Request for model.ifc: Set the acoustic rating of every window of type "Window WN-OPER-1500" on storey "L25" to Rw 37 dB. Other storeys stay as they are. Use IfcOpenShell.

First a look at what the model holds.

```python
import ifcopenshell
import ifcopenshell.util.element

model = ifcopenshell.open("model.ifc")
print(model.schema)
storey = next(s for s in model.by_type("IfcBuildingStorey") if s.Name == "L25")
windows = [e for e in ifcopenshell.util.element.get_decomposition(storey) if e.is_a("IfcWindow")]
seen = {}
for e in windows:
    element_type = ifcopenshell.util.element.get_type(e)
    key = (element_type.Name if element_type != e and element_type else None, ifcopenshell.util.element.get_pset(e, "Pset_WindowCommon", "AcousticRating"))
    seen[key] = seen.get(key, 0) + 1
for (name, value), count in sorted(seen.items(), key=str):
    print(count, "x", name, "|", value)
```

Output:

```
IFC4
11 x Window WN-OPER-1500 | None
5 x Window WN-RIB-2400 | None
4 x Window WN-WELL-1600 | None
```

```python
import ifcopenshell
import ifcopenshell.api.pset
import ifcopenshell.util.element

model = ifcopenshell.open("model.ifc")

storey = next(s for s in model.by_type("IfcBuildingStorey") if s.Name == "L25")
windows = [e for e in ifcopenshell.util.element.get_decomposition(storey) if e.is_a("IfcWindow")]

count = 0
for e in windows:
    element_type = ifcopenshell.util.element.get_type(e)
    if element_type in (None, e) or element_type.Name != "Window WN-OPER-1500":
        continue
    found = ifcopenshell.util.element.get_pset(e, "Pset_WindowCommon", should_inherit=False)
    if found:
        pset = model.by_id(found["id"])
        if len(ifcopenshell.util.element.get_elements_by_pset(pset)) > 1:
            pset = ifcopenshell.api.pset.unshare_pset(model, products=[e], pset=pset)[0]
    else:
        pset = ifcopenshell.api.pset.add_pset(model, product=e, name="Pset_WindowCommon")
    ifcopenshell.api.pset.edit_pset(model, pset=pset, properties={"AcousticRating": "Rw 37 dB"})
    count += 1

print(count, "windows updated")

model.write("model_edited.ifc")
```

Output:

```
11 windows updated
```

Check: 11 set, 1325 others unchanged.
